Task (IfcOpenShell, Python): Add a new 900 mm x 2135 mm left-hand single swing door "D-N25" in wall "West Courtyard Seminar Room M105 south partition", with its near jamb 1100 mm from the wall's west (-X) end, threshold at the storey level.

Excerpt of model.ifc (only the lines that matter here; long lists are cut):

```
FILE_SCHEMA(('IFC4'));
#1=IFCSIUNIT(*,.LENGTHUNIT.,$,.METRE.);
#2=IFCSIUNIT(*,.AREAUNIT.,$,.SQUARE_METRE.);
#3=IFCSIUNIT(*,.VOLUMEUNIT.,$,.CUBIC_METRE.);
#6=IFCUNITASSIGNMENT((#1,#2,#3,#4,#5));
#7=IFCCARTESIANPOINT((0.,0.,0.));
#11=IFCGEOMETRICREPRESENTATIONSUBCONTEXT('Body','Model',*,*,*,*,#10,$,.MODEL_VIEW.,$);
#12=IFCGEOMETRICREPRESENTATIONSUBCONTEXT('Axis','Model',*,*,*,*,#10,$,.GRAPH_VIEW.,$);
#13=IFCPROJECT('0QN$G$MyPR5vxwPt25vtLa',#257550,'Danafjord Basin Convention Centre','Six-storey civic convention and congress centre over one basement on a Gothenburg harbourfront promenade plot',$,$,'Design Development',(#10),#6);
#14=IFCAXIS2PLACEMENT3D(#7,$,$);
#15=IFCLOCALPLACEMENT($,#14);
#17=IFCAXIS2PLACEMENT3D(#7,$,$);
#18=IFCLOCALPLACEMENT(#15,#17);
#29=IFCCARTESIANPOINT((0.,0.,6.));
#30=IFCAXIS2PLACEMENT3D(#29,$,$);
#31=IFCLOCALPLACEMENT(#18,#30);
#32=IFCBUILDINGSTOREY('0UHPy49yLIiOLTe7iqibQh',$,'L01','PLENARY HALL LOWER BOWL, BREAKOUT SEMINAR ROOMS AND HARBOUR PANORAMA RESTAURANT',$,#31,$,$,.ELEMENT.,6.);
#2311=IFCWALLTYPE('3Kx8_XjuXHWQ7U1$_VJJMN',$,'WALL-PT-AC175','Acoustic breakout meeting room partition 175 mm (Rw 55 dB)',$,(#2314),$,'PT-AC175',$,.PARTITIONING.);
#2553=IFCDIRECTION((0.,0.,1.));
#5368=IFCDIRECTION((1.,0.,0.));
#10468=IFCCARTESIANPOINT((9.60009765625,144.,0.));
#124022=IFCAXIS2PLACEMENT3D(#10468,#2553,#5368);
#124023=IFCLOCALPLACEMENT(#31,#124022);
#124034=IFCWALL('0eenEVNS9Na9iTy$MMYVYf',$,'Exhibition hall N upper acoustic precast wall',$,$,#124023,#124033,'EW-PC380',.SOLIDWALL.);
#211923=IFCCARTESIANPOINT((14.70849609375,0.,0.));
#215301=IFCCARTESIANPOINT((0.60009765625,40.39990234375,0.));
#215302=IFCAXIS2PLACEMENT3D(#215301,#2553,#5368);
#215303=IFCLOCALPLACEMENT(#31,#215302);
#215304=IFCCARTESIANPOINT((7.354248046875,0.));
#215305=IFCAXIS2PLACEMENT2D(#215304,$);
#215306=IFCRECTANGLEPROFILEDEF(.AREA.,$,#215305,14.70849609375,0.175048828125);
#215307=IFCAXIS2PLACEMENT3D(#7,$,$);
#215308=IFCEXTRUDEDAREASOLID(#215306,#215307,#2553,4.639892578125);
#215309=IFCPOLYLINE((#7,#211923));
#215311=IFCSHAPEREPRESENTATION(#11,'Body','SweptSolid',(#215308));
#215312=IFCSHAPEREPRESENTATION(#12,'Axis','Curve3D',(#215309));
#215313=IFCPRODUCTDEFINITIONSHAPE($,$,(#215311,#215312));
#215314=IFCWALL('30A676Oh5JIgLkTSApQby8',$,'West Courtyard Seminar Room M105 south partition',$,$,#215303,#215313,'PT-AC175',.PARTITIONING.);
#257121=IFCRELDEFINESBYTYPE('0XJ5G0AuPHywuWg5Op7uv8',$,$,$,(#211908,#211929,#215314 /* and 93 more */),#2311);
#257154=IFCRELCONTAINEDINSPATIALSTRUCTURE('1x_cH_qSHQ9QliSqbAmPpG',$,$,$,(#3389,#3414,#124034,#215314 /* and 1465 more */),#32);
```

```python
import numpy as np
import ifcopenshell
import ifcopenshell.api.feature
import ifcopenshell.api.geometry
import ifcopenshell.api.root
import ifcopenshell.api.spatial
import ifcopenshell.geom
import ifcopenshell.util.element
import ifcopenshell.util.placement
import ifcopenshell.util.representation
import ifcopenshell.util.shape
import ifcopenshell.util.unit

model = ifcopenshell.open("model.ifc")
unit_scale = ifcopenshell.util.unit.calculate_unit_scale(model)
settings = ifcopenshell.geom.settings()


def volume(element):
    """Net volume in cubic metres, openings subtracted."""
    shape = ifcopenshell.geom.create_shape(settings, element)
    return ifcopenshell.util.shape.get_volume(shape.geometry)


wall = model.by_id(215314)
storey = ifcopenshell.util.element.get_container(wall, ifc_class="IfcBuildingStorey")
context = ifcopenshell.util.representation.get_context(model, "Model", "Body", "MODEL_VIEW")
before = volume(wall)

width, height, from_end, sill = 0.9, 2.135, 1.1, 0.0  # metres

# The wall runs along its own X axis, and the end named is its -X end.
wall_shape = ifcopenshell.geom.create_shape(settings, wall)
x, y, z = ifcopenshell.util.shape.get_vertices(wall_shape.geometry).T
start = x.min() + from_end
face, thickness = float(y.min()), float(y.max() - y.min())
wall_matrix = ifcopenshell.util.placement.get_local_placement(wall.ObjectPlacement)
level = ifcopenshell.util.placement.get_local_placement(storey.ObjectPlacement)[2, 3]


def in_wall(x, y):
    """Placement at x, y metres in the wall's axes, at sill height."""
    matrix = wall_matrix.copy()
    matrix[:, 3] = wall_matrix @ np.array([x / unit_scale, y / unit_scale, 0.0, 1.0])
    matrix[2, 3] = level + sill / unit_scale
    return matrix


# Opening: a box that overshoots both wall faces by 50 mm.
opening = ifcopenshell.api.root.create_entity(model, ifc_class="IfcOpeningElement", predefined_type="OPENING")
box = ifcopenshell.api.geometry.add_wall_representation(
    model, context=context, length=width, height=height, thickness=thickness + 0.1
)
ifcopenshell.api.geometry.assign_representation(model, product=opening, representation=box)
ifcopenshell.api.geometry.edit_object_placement(model, product=opening, matrix=in_wall(start, face - 0.05), is_si=False)
ifcopenshell.api.feature.add_feature(model, feature=opening, element=wall)

door = ifcopenshell.api.root.create_entity(model, ifc_class="IfcDoor", name="D-N25", predefined_type="DOOR")
door.OverallWidth, door.OverallHeight = width / unit_scale, height / unit_scale
door.OperationType = "SINGLE_SWING_LEFT"
body = ifcopenshell.api.geometry.add_door_representation(
    model,
    context=context,
    overall_width=door.OverallWidth,
    overall_height=door.OverallHeight,
    operation_type="SINGLE_SWING_LEFT",
    lining_properties={"LiningDepth": thickness / unit_scale, "ThresholdDepth": thickness / unit_scale},
)
ifcopenshell.api.geometry.assign_representation(model, product=door, representation=body)
ifcopenshell.api.spatial.assign_container(model, products=[door], relating_structure=storey)
ifcopenshell.api.feature.add_filling(model, opening=opening, element=door)

# The lining spans the wall, so the door starts at the wall face.
ifcopenshell.api.geometry.edit_object_placement(model, product=door, matrix=in_wall(start, face), is_si=False)

after = volume(wall)

print(f"wall volume {before:.3f} -> {after:.3f} m3")

model.write("model_v2.ifc")
```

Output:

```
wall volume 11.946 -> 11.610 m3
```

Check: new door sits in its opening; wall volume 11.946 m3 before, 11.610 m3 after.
